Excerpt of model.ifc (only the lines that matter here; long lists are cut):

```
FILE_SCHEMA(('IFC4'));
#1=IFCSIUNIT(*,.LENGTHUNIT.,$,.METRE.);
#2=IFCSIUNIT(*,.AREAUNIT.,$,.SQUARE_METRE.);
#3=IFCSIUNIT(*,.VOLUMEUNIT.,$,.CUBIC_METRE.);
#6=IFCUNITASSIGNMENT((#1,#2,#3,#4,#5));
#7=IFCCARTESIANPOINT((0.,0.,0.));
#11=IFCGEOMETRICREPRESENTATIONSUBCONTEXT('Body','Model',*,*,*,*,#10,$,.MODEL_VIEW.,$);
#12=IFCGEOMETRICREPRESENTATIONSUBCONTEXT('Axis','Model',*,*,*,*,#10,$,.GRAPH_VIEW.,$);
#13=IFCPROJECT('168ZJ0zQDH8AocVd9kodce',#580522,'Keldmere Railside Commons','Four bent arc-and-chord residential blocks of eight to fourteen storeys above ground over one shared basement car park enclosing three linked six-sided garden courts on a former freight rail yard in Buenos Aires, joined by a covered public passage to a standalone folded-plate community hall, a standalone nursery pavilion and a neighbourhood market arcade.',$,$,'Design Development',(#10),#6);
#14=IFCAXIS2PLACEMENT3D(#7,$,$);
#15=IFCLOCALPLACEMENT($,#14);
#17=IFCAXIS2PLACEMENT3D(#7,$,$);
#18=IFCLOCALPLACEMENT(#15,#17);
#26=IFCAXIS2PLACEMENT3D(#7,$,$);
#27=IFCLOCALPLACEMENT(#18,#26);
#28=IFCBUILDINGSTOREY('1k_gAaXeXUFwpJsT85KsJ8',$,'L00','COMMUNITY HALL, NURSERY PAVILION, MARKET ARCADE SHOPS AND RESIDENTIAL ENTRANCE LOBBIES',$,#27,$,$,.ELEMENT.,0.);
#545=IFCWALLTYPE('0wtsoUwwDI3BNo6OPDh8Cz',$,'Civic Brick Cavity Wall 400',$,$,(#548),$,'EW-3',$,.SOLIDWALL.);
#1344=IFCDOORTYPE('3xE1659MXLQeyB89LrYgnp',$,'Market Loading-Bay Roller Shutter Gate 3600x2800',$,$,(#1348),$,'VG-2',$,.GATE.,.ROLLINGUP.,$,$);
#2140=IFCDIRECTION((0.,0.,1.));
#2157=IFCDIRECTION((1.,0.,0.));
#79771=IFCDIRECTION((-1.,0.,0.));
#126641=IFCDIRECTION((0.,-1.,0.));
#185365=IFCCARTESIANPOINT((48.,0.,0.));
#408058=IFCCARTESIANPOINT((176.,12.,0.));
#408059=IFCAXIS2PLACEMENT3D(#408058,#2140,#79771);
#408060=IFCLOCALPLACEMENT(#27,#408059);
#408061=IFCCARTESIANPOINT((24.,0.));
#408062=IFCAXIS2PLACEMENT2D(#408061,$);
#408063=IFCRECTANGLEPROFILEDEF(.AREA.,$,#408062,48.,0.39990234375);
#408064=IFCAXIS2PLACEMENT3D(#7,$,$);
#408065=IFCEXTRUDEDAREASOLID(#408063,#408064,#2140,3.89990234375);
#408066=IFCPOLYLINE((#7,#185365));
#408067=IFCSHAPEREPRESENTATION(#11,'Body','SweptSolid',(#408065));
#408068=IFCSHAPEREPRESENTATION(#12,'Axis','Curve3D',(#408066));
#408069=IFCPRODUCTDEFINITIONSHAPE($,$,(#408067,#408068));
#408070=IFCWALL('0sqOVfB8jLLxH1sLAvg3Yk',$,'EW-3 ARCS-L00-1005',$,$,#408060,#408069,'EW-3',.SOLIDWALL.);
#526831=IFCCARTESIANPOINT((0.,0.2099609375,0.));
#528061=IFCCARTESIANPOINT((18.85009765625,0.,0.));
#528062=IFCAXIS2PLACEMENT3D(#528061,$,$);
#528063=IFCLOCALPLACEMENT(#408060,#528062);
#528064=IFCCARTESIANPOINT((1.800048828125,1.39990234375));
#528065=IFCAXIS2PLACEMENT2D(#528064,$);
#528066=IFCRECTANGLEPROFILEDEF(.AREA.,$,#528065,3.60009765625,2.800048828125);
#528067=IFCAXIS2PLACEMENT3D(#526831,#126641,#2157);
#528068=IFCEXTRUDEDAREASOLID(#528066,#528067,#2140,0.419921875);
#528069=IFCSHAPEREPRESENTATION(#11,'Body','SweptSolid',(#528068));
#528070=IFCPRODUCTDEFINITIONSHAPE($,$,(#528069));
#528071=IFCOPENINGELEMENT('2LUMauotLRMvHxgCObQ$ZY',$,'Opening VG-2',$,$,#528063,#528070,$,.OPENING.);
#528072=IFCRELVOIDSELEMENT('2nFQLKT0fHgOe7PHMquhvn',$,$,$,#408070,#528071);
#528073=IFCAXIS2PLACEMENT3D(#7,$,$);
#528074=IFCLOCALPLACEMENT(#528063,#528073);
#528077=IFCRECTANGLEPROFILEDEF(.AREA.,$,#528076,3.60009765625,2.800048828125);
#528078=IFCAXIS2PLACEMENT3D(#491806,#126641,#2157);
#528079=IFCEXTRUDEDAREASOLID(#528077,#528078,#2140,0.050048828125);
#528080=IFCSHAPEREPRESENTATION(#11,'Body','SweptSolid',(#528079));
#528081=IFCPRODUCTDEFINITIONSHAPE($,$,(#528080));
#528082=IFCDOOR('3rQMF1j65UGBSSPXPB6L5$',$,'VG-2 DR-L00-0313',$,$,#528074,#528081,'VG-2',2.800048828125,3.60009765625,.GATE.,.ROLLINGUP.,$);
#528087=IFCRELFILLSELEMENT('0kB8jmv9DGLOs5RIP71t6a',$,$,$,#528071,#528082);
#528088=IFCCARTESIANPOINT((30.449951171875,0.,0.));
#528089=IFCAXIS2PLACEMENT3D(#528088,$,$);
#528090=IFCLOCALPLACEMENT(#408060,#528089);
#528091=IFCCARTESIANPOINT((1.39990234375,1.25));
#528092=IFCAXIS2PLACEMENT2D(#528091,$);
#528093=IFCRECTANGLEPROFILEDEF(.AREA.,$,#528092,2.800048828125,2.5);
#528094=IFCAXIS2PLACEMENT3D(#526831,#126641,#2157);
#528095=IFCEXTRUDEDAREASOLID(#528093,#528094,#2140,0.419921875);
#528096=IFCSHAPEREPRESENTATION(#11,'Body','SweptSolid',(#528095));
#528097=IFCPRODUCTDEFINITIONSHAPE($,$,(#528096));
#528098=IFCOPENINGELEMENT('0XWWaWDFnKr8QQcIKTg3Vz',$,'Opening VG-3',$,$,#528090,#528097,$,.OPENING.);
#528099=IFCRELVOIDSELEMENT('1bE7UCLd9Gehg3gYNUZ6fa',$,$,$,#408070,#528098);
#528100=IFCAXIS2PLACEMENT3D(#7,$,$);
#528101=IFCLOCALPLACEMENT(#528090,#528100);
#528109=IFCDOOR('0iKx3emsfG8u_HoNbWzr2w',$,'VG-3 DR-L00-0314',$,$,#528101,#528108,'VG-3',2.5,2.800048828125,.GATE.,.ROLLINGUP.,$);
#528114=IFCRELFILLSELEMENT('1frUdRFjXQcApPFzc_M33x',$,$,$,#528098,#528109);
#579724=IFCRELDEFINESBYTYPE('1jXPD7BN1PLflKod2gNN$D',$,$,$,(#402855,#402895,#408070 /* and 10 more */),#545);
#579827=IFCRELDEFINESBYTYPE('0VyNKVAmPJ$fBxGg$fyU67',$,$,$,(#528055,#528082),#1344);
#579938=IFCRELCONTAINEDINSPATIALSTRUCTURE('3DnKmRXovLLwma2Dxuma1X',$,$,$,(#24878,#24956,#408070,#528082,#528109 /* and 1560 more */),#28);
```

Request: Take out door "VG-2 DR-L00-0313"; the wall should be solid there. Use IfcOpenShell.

```python
import ifcopenshell
import ifcopenshell.api.feature
import ifcopenshell.api.root
import ifcopenshell.geom
import ifcopenshell.util.shape

model = ifcopenshell.open("model.ifc")
settings = ifcopenshell.geom.settings()


def volume(element):
    """Net volume in cubic metres, openings subtracted."""
    shape = ifcopenshell.geom.create_shape(settings, element)
    return ifcopenshell.util.shape.get_volume(shape.geometry)


door = model.by_guid("3rQMF1j65UGBSSPXPB6L5$")
opening = door.FillsVoids[0].RelatingOpeningElement
wall = opening.VoidsElements[0].RelatingBuildingElement
before = volume(wall)

ifcopenshell.api.root.remove_product(model, product=door)
ifcopenshell.api.feature.remove_feature(model, feature=opening)

after = volume(wall)

print(f"wall volume {before:.3f} -> {after:.3f} m3")

model.write("model_rev.ifc")
```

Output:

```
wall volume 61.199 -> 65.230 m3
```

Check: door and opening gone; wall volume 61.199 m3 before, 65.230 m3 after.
